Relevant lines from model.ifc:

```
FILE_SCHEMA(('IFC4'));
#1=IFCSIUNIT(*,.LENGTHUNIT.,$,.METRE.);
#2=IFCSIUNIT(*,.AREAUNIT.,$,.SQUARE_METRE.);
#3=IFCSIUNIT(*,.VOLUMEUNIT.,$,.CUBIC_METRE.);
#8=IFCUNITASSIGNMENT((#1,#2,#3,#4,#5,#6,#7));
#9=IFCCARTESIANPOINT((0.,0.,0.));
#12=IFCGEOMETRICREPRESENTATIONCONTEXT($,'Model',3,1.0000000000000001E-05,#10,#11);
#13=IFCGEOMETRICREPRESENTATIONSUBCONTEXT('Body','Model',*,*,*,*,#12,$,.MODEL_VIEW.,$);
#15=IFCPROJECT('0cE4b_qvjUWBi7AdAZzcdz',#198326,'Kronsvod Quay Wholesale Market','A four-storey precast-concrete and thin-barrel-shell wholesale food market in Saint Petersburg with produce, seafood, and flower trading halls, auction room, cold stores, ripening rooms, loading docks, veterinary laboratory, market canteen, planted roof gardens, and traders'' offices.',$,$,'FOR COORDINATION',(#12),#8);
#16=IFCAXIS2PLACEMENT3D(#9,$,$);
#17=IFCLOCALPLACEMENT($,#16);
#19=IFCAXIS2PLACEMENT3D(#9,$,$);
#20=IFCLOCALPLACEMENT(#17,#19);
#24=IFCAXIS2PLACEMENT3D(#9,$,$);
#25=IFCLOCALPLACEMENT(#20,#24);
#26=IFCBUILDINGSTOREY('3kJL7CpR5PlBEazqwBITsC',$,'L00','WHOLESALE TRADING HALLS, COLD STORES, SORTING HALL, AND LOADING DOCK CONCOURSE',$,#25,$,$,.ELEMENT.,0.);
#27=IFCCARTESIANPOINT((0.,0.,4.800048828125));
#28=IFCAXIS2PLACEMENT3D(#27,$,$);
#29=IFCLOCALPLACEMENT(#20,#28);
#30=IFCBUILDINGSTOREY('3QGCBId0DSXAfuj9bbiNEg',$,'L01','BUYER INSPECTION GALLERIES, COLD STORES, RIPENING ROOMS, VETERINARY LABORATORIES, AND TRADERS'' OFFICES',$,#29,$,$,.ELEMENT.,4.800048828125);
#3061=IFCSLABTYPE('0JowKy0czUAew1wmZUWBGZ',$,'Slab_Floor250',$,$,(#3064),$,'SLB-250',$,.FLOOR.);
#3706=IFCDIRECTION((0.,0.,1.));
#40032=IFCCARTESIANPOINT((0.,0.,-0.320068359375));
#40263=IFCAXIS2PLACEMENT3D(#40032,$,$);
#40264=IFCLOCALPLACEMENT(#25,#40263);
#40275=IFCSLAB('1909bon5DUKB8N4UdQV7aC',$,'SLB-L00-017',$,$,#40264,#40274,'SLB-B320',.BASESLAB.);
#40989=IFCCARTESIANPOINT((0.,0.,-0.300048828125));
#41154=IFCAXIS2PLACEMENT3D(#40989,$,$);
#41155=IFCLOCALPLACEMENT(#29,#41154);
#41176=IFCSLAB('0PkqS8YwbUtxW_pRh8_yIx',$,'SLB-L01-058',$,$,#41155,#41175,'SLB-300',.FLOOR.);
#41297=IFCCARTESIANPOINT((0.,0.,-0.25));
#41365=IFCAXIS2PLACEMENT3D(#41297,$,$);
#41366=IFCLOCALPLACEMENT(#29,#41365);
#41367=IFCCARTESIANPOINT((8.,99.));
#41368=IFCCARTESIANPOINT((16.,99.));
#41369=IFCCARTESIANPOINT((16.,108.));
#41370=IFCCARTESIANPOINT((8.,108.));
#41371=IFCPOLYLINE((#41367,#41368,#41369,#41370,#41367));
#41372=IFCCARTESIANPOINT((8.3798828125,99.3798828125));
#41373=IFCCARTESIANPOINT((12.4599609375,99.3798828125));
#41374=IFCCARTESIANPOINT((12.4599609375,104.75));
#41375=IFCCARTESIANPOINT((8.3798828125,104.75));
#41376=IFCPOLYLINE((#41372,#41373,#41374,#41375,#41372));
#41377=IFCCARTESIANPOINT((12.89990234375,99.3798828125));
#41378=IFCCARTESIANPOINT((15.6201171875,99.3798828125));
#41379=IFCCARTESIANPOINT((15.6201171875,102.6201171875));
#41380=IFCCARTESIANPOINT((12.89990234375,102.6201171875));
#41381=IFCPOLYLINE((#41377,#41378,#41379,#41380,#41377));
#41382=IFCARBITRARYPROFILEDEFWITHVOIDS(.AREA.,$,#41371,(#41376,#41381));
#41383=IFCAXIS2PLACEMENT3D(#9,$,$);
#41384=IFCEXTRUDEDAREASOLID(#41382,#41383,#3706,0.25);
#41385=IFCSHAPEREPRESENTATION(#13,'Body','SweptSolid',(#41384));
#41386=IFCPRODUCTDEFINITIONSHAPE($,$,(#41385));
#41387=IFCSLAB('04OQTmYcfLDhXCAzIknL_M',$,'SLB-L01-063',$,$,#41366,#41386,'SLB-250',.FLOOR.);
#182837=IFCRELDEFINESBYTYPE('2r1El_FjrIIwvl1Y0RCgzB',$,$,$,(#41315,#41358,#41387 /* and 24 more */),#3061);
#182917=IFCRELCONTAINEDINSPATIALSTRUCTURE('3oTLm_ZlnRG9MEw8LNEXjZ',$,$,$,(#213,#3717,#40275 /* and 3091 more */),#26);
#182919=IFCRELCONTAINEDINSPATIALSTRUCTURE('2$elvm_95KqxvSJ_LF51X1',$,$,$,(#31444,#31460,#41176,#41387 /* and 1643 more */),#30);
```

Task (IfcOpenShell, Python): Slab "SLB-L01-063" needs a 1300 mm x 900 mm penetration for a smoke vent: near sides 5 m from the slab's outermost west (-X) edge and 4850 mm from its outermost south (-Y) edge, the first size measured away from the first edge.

```python
import numpy as np
import ifcopenshell
import ifcopenshell.api.feature
import ifcopenshell.api.geometry
import ifcopenshell.api.root
import ifcopenshell.geom
import ifcopenshell.util.placement
import ifcopenshell.util.representation
import ifcopenshell.util.shape
import ifcopenshell.util.unit

model = ifcopenshell.open("model.ifc")
unit_scale = ifcopenshell.util.unit.calculate_unit_scale(model)
settings = ifcopenshell.geom.settings()


def volume(element):
    """Net volume in cubic metres, openings subtracted."""
    shape = ifcopenshell.geom.create_shape(settings, element)
    return ifcopenshell.util.shape.get_volume(shape.geometry)


slab = model.by_guid("04OQTmYcfLDhXCAzIknL_M")
before = volume(slab)

# Extent in the slab's own axes, in metres. The edges named are its -X and -Y sides.
slab_shape = ifcopenshell.geom.create_shape(settings, slab)
vertices = ifcopenshell.util.shape.get_vertices(slab_shape.geometry)
x_min, y_min, bottom = vertices.min(axis=0)
top = vertices[:, 2].max()

opening = ifcopenshell.api.root.create_entity(model, ifc_class="IfcOpeningElement", name="Smoke vent opening", predefined_type="OPENING")
context = ifcopenshell.util.representation.get_context(model, "Model", "Body", "MODEL_VIEW")
width, depth = 1.3, 0.9
outline = [(0.0, 0.0), (width, 0.0), (width, depth), (0.0, depth), (0.0, 0.0)]
# Overshoot both faces by 50 mm so the cut is clean.
shape = ifcopenshell.api.geometry.add_slab_representation(
    model, context=context, depth=top - bottom + 0.1, polyline=outline
)
ifcopenshell.api.geometry.assign_representation(model, product=opening, representation=shape)

matrix = ifcopenshell.util.placement.get_local_placement(slab.ObjectPlacement)
matrix[:, 3] = matrix @ np.append(np.array([x_min + 5, y_min + 4.85, bottom - 0.05]) / unit_scale, 1.0)
ifcopenshell.api.geometry.edit_object_placement(model, product=opening, matrix=matrix, is_si=False)
ifcopenshell.api.feature.add_feature(model, feature=opening, element=slab)

after = volume(slab)

print(f"slab volume {before:.3f} -> {after:.3f} m3")

model.write("model_edited.ifc")
```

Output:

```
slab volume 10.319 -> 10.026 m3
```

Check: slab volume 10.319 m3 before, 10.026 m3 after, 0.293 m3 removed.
